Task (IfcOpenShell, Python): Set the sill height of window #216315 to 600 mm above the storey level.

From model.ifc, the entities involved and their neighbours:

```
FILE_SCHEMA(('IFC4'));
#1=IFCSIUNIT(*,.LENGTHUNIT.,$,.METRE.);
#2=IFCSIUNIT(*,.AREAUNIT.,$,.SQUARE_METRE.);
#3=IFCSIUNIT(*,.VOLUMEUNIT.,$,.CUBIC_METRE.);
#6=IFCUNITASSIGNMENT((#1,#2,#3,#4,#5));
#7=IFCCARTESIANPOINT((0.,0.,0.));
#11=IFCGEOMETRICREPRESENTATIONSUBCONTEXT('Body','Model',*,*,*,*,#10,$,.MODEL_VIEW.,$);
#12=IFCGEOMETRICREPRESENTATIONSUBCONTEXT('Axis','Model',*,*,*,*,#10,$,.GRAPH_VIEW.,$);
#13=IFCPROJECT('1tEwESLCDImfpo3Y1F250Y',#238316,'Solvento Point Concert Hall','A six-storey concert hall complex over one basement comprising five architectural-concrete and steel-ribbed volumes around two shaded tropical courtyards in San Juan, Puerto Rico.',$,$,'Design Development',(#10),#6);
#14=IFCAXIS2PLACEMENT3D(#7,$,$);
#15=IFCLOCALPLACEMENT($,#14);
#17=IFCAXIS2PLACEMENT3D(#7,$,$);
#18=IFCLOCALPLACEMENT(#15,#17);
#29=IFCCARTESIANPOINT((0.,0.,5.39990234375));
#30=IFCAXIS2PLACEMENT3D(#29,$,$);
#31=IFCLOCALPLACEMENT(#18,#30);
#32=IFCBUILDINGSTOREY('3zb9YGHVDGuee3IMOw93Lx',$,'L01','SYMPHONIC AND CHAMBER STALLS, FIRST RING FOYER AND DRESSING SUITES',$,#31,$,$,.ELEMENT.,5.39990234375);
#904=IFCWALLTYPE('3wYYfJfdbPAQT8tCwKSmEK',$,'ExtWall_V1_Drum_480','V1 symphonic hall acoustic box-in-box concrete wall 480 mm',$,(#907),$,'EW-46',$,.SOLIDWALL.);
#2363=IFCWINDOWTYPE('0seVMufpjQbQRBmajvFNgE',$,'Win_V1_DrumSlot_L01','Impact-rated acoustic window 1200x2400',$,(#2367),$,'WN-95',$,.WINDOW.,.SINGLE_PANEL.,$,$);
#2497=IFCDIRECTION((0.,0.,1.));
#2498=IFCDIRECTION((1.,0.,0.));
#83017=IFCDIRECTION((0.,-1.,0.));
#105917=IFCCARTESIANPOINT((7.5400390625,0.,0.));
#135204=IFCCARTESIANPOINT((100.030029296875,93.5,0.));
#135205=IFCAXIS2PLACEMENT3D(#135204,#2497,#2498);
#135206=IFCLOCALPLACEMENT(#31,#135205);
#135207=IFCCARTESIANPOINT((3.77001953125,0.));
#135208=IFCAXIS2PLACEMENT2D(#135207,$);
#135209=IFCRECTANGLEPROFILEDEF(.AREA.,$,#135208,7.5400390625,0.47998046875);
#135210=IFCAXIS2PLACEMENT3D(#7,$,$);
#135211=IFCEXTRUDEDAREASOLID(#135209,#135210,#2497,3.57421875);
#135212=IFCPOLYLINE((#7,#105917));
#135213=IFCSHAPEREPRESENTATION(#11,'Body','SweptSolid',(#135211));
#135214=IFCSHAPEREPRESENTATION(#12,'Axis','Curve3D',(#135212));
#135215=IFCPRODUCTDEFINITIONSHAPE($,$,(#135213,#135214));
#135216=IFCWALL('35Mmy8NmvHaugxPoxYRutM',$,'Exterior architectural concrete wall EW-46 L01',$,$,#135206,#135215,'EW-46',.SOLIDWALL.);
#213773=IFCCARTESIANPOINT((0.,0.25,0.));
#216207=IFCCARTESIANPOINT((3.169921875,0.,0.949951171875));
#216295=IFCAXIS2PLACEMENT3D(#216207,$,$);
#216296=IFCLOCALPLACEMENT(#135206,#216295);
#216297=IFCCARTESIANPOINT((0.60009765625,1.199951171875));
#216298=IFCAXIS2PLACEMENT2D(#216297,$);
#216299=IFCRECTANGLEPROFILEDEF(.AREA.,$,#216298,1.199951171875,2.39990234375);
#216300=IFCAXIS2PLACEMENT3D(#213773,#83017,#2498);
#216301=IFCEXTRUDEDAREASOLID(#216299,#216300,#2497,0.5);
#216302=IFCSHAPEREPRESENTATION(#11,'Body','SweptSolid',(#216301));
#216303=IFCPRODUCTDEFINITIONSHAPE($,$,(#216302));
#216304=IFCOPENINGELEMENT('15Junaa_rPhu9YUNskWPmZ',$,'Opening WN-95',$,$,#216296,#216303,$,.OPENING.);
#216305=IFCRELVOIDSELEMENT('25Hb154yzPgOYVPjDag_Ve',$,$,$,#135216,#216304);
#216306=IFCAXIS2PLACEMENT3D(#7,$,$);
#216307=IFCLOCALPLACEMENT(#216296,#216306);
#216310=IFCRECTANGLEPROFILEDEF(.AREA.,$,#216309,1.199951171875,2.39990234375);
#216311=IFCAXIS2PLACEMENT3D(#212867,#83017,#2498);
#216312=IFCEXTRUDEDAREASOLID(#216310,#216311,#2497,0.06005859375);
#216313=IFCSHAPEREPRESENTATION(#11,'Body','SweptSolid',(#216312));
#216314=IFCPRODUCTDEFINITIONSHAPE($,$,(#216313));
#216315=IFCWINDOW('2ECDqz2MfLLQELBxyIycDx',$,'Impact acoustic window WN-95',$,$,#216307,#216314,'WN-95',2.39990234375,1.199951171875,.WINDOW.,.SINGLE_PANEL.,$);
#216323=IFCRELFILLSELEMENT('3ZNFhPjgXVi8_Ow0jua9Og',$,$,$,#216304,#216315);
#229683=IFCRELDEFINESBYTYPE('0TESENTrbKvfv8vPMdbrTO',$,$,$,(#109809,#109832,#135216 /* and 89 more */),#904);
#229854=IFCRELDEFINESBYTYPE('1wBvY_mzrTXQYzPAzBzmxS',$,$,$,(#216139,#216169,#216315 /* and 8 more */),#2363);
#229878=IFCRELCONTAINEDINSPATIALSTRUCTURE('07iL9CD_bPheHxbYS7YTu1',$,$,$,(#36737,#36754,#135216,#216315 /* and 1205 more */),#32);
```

```python
import numpy as np
import ifcopenshell
import ifcopenshell.api.geometry
import ifcopenshell.geom
import ifcopenshell.util.element
import ifcopenshell.util.placement
import ifcopenshell.util.shape
import ifcopenshell.util.unit

model = ifcopenshell.open("model.ifc")
unit_scale = ifcopenshell.util.unit.calculate_unit_scale(model)

window = model.by_id(216315)
opening = window.FillsVoids[0].RelatingOpeningElement
storey = ifcopenshell.util.element.get_container(window, ifc_class="IfcBuildingStorey")
level = ifcopenshell.util.placement.get_local_placement(storey.ObjectPlacement)[2, 3]

# The opening's origin need not be at the sill, so measure its lowest point.
shape = ifcopenshell.geom.create_shape(ifcopenshell.geom.settings(), opening)
bottom = ifcopenshell.util.shape.get_shape_bottom_elevation(shape, shape.geometry) / unit_scale
dz = level + 0.6 - bottom

shift = np.array([0.0, 0.0, dz])
# The window is placed relative to its opening, so it follows when the opening moves.
matrix = ifcopenshell.util.placement.get_local_placement(opening.ObjectPlacement)
matrix[:3, 3] += shift
ifcopenshell.api.geometry.edit_object_placement(
    model, product=opening, matrix=matrix, is_si=False, should_transform_children=True
)

print(f"moved by {dz * unit_scale:+.3f} m")

model.write("model_v2.ifc")
```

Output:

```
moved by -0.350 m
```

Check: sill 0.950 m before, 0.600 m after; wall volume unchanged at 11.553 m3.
